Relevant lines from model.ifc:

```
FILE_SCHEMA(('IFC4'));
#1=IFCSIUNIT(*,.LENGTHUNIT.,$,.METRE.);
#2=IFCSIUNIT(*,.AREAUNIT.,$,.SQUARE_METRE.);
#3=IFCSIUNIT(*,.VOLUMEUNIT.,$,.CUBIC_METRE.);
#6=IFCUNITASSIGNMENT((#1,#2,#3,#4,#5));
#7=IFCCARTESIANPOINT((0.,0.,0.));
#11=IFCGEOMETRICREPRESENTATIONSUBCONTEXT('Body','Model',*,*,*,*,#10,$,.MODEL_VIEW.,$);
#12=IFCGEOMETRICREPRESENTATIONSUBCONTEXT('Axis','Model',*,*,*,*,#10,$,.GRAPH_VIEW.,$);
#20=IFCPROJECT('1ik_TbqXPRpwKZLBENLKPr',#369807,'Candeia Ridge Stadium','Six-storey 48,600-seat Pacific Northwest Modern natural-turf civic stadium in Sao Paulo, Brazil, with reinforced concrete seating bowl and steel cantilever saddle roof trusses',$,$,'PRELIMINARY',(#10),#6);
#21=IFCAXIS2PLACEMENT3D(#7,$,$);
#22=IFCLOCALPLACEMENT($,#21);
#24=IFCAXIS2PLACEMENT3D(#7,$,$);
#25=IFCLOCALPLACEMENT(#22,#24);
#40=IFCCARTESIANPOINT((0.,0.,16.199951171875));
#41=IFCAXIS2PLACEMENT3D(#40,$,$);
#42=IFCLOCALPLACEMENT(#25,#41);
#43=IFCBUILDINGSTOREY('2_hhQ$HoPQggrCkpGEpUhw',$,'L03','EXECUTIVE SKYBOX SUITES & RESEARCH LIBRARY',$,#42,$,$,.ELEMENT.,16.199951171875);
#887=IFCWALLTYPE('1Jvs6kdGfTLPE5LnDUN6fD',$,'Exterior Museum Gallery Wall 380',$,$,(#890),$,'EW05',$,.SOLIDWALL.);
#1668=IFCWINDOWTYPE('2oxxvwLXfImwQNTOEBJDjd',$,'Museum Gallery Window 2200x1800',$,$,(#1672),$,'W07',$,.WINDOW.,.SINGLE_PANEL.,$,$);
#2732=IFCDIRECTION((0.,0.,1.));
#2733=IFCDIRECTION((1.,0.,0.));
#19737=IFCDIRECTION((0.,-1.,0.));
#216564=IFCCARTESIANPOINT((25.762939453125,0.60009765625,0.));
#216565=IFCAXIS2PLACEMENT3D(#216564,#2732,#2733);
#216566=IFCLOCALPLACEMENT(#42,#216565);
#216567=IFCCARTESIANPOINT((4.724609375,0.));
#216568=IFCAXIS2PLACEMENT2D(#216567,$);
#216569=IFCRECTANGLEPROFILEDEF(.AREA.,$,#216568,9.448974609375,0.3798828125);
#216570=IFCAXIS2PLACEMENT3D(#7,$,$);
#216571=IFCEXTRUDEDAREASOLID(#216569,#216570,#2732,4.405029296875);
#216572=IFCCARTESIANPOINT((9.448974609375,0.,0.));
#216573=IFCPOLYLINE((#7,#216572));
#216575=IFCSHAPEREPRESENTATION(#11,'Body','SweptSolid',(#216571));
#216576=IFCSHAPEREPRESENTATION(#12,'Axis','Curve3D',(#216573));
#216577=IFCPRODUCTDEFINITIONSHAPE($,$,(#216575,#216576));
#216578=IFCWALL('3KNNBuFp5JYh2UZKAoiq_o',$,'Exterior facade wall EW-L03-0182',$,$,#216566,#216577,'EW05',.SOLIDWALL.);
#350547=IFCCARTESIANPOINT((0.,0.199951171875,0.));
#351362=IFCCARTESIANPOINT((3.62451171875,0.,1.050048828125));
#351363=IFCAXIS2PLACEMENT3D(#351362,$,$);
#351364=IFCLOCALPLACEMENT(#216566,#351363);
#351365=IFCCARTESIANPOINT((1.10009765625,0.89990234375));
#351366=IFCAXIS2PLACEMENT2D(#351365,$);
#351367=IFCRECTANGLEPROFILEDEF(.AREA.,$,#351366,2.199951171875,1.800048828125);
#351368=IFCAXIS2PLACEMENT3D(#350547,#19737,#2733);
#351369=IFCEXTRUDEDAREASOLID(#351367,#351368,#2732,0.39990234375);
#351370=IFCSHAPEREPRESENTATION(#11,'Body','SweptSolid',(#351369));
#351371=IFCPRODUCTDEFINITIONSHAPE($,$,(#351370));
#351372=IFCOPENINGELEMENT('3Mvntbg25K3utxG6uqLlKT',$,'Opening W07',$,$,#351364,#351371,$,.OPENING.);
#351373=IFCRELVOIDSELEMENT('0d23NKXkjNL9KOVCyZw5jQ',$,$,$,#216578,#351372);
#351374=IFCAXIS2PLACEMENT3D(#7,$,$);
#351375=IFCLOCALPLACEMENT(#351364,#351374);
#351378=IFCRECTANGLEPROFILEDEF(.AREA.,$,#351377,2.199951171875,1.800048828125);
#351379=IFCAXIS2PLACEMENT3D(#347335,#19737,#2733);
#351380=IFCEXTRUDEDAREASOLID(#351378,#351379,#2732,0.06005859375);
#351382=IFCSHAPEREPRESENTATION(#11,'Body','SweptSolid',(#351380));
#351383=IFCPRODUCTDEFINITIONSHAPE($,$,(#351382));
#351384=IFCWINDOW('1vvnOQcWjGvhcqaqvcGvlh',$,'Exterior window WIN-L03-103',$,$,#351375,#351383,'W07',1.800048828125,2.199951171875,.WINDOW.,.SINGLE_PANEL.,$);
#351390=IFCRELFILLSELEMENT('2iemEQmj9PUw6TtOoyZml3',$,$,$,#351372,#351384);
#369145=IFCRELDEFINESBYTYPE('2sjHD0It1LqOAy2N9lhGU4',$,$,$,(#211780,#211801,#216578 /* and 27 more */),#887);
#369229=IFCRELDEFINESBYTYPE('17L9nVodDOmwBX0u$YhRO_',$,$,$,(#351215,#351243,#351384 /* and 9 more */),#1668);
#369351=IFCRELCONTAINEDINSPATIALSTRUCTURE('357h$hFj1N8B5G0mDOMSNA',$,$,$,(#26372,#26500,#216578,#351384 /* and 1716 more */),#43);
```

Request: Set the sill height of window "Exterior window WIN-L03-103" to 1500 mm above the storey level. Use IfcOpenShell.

```python
import numpy as np
import ifcopenshell
import ifcopenshell.api.geometry
import ifcopenshell.geom
import ifcopenshell.util.element
import ifcopenshell.util.placement
import ifcopenshell.util.shape
import ifcopenshell.util.unit

model = ifcopenshell.open("model.ifc")
unit_scale = ifcopenshell.util.unit.calculate_unit_scale(model)

window = model.by_guid("1vvnOQcWjGvhcqaqvcGvlh")
opening = window.FillsVoids[0].RelatingOpeningElement
storey = ifcopenshell.util.element.get_container(window, ifc_class="IfcBuildingStorey")
level = ifcopenshell.util.placement.get_local_placement(storey.ObjectPlacement)[2, 3]

# The opening's origin need not be at the sill, so measure its lowest point.
shape = ifcopenshell.geom.create_shape(ifcopenshell.geom.settings(), opening)
bottom = ifcopenshell.util.shape.get_shape_bottom_elevation(shape, shape.geometry) / unit_scale
dz = level + 1.5 / unit_scale - bottom

shift = np.array([0.0, 0.0, dz])
# The window is placed relative to its opening, so it follows when the opening moves.
matrix = ifcopenshell.util.placement.get_local_placement(opening.ObjectPlacement)
matrix[:3, 3] += shift
ifcopenshell.api.geometry.edit_object_placement(
    model, product=opening, matrix=matrix, is_si=False, should_transform_children=True
)

print(f"moved by {dz * unit_scale:+.3f} m")

model.write("model_rev.ifc")
```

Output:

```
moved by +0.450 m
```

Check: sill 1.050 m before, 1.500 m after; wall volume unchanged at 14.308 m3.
